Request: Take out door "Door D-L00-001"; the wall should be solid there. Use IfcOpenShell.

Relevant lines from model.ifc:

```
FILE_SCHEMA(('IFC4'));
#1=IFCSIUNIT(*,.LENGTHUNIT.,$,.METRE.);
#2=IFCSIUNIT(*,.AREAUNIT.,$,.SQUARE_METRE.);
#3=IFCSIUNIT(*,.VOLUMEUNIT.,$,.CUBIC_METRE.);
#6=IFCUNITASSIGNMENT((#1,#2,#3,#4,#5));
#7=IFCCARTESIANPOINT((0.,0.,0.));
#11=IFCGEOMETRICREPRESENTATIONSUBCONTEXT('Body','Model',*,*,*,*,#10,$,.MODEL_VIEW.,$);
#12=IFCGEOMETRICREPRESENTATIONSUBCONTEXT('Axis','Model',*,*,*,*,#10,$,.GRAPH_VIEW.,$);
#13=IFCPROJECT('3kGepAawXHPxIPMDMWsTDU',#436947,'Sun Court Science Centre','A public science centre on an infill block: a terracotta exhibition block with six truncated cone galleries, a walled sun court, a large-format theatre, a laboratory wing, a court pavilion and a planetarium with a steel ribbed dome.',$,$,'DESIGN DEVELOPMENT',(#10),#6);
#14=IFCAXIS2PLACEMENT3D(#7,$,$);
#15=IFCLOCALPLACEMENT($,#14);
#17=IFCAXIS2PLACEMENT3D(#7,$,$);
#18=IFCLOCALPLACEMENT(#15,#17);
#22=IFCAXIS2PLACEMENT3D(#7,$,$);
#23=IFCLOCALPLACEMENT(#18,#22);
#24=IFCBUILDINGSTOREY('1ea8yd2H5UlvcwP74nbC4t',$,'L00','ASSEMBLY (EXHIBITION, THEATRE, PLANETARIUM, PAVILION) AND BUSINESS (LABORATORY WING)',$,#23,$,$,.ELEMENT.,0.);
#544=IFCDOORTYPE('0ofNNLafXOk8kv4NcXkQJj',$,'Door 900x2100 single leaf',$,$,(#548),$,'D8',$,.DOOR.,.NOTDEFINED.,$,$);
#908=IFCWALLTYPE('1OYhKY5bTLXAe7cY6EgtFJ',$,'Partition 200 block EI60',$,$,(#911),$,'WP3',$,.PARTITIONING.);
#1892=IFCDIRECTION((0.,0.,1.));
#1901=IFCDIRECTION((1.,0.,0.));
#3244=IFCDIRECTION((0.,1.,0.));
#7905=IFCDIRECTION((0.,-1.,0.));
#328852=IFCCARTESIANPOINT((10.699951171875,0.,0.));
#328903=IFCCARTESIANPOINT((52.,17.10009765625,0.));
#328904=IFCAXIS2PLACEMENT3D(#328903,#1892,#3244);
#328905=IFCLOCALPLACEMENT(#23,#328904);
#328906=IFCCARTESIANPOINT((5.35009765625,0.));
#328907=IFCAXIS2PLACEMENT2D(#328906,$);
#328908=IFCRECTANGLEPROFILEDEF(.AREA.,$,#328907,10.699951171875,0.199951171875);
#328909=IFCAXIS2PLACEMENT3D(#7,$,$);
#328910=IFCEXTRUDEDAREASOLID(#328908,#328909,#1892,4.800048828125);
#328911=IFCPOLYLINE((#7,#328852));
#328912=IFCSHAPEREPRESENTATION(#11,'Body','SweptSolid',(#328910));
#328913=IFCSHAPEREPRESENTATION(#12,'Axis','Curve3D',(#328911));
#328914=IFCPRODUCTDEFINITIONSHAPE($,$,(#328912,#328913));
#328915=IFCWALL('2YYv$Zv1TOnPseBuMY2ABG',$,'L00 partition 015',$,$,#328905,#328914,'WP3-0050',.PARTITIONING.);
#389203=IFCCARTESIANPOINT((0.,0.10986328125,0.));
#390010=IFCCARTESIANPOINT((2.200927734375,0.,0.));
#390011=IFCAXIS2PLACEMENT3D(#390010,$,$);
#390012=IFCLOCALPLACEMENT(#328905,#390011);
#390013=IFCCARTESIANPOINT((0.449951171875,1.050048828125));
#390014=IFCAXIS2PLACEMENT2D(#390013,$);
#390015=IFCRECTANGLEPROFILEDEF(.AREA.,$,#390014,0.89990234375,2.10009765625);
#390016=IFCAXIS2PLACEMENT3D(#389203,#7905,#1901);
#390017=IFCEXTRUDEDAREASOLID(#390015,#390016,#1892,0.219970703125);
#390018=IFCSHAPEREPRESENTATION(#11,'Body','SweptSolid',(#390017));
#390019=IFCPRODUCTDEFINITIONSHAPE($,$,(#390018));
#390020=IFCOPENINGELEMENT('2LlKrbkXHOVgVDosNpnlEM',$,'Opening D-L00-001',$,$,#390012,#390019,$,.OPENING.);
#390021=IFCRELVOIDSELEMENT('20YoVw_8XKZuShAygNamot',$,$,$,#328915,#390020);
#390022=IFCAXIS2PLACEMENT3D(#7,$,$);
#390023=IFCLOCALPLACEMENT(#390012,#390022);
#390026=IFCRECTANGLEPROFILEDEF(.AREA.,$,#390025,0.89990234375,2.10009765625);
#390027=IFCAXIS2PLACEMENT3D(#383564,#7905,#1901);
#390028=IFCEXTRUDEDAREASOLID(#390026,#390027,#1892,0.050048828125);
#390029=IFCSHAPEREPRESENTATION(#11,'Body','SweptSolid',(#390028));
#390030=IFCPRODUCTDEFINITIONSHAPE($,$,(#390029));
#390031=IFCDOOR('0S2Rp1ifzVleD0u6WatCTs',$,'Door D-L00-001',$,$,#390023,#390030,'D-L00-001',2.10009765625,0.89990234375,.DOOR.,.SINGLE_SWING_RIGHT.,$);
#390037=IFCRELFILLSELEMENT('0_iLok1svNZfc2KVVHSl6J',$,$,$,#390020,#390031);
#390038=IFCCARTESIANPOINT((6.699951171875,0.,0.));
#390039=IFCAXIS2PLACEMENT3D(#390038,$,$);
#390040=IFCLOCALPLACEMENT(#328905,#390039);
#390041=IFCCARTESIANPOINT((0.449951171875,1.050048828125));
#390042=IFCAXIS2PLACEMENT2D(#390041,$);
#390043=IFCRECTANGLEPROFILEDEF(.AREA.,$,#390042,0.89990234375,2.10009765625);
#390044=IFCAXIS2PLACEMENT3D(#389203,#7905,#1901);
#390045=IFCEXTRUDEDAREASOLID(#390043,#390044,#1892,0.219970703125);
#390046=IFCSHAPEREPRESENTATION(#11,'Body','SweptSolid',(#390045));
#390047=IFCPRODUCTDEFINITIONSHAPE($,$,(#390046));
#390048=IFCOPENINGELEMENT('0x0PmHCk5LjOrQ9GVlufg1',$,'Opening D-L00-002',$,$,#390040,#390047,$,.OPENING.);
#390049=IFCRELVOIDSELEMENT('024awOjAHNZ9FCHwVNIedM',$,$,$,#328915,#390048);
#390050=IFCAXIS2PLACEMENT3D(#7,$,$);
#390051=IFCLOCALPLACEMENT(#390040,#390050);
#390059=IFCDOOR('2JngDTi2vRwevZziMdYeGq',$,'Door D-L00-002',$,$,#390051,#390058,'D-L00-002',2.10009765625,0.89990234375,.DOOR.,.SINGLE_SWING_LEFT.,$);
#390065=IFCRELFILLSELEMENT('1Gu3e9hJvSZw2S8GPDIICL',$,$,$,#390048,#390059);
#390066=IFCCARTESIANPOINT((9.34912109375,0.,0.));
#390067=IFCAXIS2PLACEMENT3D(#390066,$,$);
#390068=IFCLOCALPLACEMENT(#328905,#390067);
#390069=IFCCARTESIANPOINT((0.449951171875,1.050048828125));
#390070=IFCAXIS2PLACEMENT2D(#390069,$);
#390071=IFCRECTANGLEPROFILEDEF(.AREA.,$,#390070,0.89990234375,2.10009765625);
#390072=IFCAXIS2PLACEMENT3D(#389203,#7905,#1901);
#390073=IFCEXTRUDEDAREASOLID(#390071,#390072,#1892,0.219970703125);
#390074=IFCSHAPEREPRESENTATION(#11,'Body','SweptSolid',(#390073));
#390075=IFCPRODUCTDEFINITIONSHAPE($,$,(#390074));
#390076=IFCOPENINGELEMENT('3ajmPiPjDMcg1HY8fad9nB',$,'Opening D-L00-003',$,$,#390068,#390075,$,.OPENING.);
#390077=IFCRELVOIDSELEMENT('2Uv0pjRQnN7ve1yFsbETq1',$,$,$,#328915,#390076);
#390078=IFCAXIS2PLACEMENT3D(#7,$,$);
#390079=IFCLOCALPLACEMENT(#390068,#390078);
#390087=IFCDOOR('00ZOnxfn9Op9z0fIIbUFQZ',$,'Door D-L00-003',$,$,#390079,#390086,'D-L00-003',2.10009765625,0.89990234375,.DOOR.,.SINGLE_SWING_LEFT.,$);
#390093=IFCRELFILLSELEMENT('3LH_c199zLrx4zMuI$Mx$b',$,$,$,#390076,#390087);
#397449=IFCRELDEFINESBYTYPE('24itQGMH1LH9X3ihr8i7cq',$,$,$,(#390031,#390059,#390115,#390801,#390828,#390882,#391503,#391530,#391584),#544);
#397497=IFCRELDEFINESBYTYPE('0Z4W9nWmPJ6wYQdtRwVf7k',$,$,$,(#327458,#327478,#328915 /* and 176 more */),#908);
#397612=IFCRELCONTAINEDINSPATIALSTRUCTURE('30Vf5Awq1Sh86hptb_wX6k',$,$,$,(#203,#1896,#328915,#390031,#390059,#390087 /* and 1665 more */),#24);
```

```python
import ifcopenshell
import ifcopenshell.api.feature
import ifcopenshell.api.root
import ifcopenshell.geom
import ifcopenshell.util.shape

model = ifcopenshell.open("model.ifc")
settings = ifcopenshell.geom.settings()


def volume(element):
    """Net volume in cubic metres, openings subtracted."""
    shape = ifcopenshell.geom.create_shape(settings, element)
    return ifcopenshell.util.shape.get_volume(shape.geometry)


door = model.by_guid("0S2Rp1ifzVleD0u6WatCTs")
opening = door.FillsVoids[0].RelatingOpeningElement
wall = opening.VoidsElements[0].RelatingBuildingElement
before = volume(wall)

ifcopenshell.api.root.remove_product(model, product=door)
ifcopenshell.api.feature.remove_feature(model, feature=opening)

after = volume(wall)

print(f"wall volume {before:.3f} -> {after:.3f} m3")

model.write("model_updated.ifc")
```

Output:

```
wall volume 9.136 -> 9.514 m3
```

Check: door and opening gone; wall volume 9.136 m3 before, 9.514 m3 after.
